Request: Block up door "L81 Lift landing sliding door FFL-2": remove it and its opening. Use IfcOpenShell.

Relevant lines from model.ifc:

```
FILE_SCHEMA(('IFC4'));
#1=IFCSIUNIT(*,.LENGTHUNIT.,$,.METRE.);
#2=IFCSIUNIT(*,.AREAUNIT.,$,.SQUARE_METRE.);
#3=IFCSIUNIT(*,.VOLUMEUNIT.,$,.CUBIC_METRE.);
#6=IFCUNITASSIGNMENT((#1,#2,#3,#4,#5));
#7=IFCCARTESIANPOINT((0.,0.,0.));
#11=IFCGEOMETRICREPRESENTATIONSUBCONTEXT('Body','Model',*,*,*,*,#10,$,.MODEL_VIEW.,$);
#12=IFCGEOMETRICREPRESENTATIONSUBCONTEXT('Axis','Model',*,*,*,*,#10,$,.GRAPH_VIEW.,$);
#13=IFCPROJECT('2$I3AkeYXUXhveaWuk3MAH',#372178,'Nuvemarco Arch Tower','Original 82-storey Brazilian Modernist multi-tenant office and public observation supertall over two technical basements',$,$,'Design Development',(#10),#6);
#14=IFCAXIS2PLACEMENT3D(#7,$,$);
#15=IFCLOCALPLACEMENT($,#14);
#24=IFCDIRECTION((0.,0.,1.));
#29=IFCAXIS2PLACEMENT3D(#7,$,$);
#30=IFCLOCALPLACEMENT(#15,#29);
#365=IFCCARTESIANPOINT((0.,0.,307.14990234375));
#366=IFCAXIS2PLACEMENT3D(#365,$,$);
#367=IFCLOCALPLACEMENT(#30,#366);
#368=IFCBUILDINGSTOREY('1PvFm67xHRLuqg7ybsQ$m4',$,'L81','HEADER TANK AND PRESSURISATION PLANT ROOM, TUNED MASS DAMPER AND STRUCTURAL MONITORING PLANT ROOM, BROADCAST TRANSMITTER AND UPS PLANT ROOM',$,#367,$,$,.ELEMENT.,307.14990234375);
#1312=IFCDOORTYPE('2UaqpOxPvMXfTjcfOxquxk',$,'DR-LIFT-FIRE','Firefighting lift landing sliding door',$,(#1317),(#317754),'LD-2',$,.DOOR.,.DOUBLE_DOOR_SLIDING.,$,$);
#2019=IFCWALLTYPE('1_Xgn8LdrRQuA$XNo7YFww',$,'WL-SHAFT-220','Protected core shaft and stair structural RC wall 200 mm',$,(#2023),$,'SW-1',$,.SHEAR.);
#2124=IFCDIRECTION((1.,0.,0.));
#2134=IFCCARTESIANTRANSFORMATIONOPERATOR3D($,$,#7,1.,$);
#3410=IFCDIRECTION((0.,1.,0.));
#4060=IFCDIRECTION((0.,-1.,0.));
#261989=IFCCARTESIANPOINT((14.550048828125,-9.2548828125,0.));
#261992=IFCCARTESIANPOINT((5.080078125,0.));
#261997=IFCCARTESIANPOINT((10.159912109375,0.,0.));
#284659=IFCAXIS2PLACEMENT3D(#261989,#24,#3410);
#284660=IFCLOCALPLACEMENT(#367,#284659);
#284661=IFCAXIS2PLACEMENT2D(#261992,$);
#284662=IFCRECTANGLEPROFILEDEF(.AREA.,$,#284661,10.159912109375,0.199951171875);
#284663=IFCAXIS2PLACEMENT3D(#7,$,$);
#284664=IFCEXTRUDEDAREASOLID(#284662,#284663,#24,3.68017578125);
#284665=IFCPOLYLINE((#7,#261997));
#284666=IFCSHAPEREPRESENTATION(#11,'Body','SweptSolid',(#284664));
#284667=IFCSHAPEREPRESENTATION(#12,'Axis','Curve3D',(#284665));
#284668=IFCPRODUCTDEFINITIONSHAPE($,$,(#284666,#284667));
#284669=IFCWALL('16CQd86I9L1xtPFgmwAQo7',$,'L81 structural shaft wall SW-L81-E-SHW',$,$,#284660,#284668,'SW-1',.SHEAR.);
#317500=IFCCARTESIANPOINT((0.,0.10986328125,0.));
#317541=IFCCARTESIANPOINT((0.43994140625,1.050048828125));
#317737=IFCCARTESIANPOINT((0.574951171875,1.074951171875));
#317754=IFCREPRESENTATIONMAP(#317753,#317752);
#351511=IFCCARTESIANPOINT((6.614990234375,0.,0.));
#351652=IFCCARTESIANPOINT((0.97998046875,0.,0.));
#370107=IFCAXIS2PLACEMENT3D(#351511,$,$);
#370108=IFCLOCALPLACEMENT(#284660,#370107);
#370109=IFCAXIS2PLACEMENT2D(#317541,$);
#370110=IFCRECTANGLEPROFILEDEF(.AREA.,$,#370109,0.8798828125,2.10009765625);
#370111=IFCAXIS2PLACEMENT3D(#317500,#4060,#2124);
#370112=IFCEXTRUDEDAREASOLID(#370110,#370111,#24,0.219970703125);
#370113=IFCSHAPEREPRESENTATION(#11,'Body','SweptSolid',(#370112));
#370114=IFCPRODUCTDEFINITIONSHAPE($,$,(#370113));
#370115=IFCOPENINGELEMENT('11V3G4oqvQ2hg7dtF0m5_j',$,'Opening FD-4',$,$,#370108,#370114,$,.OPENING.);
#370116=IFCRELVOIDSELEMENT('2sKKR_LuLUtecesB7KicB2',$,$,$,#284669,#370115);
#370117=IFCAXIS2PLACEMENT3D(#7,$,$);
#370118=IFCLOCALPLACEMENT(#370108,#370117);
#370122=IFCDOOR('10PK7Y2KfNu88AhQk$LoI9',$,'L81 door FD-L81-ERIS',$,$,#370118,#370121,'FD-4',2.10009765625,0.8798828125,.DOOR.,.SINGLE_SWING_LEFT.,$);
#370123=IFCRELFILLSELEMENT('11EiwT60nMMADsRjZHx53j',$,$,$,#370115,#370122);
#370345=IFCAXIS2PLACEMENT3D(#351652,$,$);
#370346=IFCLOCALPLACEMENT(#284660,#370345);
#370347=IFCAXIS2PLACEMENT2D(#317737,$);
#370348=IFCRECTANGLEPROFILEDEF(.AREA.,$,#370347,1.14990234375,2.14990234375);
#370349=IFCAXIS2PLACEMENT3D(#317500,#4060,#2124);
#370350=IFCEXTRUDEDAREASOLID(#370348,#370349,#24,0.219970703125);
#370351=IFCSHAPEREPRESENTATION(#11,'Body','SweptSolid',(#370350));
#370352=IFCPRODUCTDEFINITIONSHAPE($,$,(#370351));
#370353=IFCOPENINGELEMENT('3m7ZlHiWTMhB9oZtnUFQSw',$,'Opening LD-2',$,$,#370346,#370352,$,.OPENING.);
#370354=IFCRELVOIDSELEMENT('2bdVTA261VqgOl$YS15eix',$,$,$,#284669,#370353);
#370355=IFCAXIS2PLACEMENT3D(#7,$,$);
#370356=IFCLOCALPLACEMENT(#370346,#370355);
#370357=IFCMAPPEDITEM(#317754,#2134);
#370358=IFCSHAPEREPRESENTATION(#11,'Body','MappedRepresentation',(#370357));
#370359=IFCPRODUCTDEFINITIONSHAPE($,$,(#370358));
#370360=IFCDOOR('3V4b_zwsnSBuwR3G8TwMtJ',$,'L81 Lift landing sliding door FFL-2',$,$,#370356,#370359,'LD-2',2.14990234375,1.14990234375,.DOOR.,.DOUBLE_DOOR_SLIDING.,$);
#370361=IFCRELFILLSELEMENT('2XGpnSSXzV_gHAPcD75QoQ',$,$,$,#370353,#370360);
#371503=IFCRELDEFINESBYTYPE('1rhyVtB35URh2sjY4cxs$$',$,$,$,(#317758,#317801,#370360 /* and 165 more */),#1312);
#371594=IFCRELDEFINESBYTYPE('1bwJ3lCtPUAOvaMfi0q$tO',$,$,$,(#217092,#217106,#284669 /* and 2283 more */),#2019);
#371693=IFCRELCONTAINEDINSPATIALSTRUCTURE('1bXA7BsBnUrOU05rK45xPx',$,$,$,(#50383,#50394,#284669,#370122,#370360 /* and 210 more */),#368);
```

```python
import ifcopenshell
import ifcopenshell.api.feature
import ifcopenshell.api.root
import ifcopenshell.geom
import ifcopenshell.util.shape

model = ifcopenshell.open("model.ifc")
settings = ifcopenshell.geom.settings()


def volume(element):
    """Net volume in cubic metres, openings subtracted."""
    shape = ifcopenshell.geom.create_shape(settings, element)
    return ifcopenshell.util.shape.get_volume(shape.geometry)


door = model.by_id(370360)
opening = door.FillsVoids[0].RelatingOpeningElement
wall = opening.VoidsElements[0].RelatingBuildingElement
before = volume(wall)

ifcopenshell.api.root.remove_product(model, product=door)
ifcopenshell.api.feature.remove_feature(model, feature=opening)

after = volume(wall)

print(f"wall volume {before:.3f} -> {after:.3f} m3")

model.write("model_rev.ifc")
```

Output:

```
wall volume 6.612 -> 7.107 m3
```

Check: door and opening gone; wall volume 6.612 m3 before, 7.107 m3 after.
